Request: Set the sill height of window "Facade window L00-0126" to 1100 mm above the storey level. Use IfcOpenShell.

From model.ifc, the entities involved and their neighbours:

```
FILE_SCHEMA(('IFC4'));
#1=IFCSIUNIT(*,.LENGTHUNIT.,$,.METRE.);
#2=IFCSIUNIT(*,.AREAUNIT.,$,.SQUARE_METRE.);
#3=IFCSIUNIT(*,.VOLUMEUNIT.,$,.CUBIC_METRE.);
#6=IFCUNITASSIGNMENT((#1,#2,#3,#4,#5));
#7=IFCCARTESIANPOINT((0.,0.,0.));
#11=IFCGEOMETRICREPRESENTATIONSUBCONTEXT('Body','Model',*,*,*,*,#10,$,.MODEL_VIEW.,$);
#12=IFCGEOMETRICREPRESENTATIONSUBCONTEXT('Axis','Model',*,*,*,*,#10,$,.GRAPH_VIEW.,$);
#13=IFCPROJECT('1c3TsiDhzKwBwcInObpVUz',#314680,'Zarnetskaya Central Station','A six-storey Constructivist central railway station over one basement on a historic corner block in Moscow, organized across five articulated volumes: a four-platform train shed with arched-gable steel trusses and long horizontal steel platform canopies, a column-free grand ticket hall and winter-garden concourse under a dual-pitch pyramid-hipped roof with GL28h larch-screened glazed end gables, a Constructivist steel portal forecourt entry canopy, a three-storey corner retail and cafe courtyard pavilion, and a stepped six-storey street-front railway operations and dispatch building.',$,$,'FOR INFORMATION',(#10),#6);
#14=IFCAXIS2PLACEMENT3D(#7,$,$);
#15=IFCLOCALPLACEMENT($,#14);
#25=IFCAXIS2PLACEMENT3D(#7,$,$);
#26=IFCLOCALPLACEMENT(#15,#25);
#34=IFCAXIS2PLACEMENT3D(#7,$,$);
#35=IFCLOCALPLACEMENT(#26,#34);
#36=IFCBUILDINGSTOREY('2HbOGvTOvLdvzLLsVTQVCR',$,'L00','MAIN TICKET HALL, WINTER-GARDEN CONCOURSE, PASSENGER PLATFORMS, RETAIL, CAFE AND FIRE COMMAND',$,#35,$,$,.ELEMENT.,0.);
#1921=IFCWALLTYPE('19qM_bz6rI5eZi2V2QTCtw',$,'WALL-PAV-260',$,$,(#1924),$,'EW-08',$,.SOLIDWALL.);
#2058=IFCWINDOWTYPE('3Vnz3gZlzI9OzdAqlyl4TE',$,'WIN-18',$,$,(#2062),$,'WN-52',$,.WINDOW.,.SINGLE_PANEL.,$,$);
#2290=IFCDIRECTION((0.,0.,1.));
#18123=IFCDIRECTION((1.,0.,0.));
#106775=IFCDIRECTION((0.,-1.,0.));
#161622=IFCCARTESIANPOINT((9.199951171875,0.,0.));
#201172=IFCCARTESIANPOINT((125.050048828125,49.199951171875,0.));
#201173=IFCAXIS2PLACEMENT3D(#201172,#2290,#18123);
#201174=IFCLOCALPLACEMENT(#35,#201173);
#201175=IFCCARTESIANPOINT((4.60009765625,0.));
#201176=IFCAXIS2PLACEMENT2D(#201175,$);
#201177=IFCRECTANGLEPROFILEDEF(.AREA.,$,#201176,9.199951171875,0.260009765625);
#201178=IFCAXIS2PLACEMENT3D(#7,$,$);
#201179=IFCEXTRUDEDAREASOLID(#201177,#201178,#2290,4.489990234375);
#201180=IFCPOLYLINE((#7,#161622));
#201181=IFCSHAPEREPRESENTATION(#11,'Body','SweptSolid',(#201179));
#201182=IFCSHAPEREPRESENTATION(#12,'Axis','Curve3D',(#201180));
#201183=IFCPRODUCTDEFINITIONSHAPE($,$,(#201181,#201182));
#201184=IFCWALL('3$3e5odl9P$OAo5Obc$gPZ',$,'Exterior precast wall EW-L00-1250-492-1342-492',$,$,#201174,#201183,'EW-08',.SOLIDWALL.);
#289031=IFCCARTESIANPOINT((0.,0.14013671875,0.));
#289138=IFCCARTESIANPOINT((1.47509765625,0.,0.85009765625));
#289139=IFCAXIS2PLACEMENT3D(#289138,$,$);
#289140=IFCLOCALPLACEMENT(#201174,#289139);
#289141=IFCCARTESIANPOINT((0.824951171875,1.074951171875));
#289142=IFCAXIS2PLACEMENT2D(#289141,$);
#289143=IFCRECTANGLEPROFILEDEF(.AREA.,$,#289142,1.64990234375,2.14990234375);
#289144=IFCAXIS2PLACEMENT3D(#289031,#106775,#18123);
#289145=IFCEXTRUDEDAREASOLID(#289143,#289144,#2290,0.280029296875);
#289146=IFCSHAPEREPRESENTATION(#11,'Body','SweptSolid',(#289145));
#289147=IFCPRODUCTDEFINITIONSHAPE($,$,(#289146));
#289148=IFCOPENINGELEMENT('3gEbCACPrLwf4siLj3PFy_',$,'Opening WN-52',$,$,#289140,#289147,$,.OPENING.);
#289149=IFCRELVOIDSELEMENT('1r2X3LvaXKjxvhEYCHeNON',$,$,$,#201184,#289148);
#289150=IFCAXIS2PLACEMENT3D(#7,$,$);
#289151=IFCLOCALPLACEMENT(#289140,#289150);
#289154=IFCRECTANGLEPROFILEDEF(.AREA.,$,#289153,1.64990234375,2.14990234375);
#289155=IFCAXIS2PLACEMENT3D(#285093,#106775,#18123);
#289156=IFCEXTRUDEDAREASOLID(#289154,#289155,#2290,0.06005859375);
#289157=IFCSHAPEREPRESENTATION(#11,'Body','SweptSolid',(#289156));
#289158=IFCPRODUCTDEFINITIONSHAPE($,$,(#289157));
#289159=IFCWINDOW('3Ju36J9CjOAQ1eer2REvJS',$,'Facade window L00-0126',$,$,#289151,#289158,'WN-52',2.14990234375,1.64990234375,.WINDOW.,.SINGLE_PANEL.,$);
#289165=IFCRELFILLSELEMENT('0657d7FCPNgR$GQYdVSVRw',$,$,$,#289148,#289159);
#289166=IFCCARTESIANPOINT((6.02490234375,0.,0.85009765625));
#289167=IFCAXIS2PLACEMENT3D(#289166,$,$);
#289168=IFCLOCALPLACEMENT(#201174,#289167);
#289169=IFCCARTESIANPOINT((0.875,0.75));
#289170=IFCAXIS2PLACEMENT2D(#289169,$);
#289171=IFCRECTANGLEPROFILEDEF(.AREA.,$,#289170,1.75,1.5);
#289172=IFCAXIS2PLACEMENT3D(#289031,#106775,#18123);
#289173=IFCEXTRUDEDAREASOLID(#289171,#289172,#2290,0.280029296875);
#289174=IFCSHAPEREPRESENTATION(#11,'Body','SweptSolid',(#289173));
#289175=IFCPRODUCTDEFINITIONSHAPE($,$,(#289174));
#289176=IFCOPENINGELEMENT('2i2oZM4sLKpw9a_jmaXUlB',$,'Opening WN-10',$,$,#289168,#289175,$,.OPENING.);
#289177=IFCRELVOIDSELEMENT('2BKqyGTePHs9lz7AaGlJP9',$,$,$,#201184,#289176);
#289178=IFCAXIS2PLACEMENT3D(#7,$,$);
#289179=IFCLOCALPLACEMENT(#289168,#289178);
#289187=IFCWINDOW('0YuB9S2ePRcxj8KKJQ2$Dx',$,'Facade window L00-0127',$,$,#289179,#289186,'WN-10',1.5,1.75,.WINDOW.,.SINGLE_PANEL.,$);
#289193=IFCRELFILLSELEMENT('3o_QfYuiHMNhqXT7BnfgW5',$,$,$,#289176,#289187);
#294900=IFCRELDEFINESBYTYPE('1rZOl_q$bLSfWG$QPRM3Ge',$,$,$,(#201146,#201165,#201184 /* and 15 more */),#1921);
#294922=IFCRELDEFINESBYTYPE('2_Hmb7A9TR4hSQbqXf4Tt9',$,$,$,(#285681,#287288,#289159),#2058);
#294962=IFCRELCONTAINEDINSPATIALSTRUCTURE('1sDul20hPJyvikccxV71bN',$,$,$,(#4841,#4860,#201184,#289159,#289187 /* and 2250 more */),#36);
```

```python
import numpy as np
import ifcopenshell
import ifcopenshell.api.geometry
import ifcopenshell.geom
import ifcopenshell.util.element
import ifcopenshell.util.placement
import ifcopenshell.util.shape
import ifcopenshell.util.unit

model = ifcopenshell.open("model.ifc")
unit_scale = ifcopenshell.util.unit.calculate_unit_scale(model)

window = model.by_guid("3Ju36J9CjOAQ1eer2REvJS")
opening = window.FillsVoids[0].RelatingOpeningElement
storey = ifcopenshell.util.element.get_container(window, ifc_class="IfcBuildingStorey")
level = ifcopenshell.util.placement.get_local_placement(storey.ObjectPlacement)[2, 3]

# The opening's origin need not be at the sill, so measure its lowest point.
shape = ifcopenshell.geom.create_shape(ifcopenshell.geom.settings(), opening)
bottom = ifcopenshell.util.shape.get_shape_bottom_elevation(shape, shape.geometry) / unit_scale
dz = level + 1.1 / unit_scale - bottom

shift = np.array([0.0, 0.0, dz])
# The window is placed relative to its opening, so it follows when the opening moves.
matrix = ifcopenshell.util.placement.get_local_placement(opening.ObjectPlacement)
matrix[:3, 3] += shift
ifcopenshell.api.geometry.edit_object_placement(
    model, product=opening, matrix=matrix, is_si=False, should_transform_children=True
)

print(f"moved by {dz * unit_scale:+.3f} m")

model.write("model-out.ifc")
```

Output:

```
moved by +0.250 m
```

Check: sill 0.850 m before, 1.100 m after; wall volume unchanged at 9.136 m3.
